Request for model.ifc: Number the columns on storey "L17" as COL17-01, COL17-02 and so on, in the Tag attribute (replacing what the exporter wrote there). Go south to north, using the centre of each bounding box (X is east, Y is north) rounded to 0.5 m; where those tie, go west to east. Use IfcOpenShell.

First a look at what the model holds.

```python
import ifcopenshell
import ifcopenshell.util.element
import ifcopenshell.util.placement

model = ifcopenshell.open("model.ifc")
print(model.schema)
storey = next(s for s in model.by_type("IfcBuildingStorey") if s.Name == "L17")
columns = [e for e in ifcopenshell.util.element.get_decomposition(storey) if e.is_a("IfcColumn")]
for e in sorted(columns, key=lambda e: e.id()):
    origin = ifcopenshell.util.placement.get_local_placement(e.ObjectPlacement)[:3, 3]
    print(e.id(), e.Tag, e.Name, origin.round(2) + 0.0, sep=" | ")
```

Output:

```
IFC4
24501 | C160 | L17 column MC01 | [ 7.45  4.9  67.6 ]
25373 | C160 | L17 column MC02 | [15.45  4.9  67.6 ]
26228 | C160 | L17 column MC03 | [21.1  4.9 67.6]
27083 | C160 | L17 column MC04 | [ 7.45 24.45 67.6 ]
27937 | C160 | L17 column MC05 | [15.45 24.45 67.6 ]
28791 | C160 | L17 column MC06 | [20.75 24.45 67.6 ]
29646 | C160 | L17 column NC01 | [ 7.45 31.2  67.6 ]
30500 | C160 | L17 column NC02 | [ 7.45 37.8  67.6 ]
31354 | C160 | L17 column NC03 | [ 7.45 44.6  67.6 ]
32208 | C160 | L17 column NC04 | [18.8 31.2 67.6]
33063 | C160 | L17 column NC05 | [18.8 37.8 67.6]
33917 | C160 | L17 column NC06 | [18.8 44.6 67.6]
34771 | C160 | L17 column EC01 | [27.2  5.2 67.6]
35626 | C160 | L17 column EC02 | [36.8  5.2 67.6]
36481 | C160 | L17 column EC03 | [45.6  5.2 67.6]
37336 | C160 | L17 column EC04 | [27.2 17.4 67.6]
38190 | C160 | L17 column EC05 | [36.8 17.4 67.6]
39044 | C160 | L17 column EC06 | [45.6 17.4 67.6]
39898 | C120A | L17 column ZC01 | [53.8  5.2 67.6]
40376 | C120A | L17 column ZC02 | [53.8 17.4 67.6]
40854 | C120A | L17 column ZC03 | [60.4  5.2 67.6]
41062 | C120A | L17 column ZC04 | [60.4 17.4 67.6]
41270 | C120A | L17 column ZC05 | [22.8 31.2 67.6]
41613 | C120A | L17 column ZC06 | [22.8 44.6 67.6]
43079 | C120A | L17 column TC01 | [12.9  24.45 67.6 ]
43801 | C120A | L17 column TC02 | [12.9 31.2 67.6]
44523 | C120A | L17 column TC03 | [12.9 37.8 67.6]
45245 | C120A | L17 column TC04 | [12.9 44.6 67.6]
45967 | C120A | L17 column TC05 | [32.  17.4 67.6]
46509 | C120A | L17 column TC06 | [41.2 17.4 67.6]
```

```python
import ifcopenshell
import ifcopenshell.geom
import ifcopenshell.util.element
import ifcopenshell.util.shape

model = ifcopenshell.open("model.ifc")
settings = ifcopenshell.geom.settings()
settings.set("use-world-coords", True)


def centre(element):
    shape = ifcopenshell.geom.create_shape(settings, element)
    return ifcopenshell.util.shape.get_bbox_centroid(shape.geometry)


storey = next(s for s in model.by_type("IfcBuildingStorey") if s.Name == "L17")
columns = [e for e in ifcopenshell.util.element.get_decomposition(storey) if e.is_a("IfcColumn")]

# Insertion points can sit at a corner or the storey origin, so sort by the geometry (in metres).
centres = {e: centre(e) for e in columns}
columns.sort(key=lambda e: (round(centres[e][1] / 0.5), centres[e][0]))

for i, e in enumerate(columns, start=1):
    number = f"COL17-{i:02d}"
    e.Tag = number
    print(e.id(), number)

model.write("model_updated.ifc")
```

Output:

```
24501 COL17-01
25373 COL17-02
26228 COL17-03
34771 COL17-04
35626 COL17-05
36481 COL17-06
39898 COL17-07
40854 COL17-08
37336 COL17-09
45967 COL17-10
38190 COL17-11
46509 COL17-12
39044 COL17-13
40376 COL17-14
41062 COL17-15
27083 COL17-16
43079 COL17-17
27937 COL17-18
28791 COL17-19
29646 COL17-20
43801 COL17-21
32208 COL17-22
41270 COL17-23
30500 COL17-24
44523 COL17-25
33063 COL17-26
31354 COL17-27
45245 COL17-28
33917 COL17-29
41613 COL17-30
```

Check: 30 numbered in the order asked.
